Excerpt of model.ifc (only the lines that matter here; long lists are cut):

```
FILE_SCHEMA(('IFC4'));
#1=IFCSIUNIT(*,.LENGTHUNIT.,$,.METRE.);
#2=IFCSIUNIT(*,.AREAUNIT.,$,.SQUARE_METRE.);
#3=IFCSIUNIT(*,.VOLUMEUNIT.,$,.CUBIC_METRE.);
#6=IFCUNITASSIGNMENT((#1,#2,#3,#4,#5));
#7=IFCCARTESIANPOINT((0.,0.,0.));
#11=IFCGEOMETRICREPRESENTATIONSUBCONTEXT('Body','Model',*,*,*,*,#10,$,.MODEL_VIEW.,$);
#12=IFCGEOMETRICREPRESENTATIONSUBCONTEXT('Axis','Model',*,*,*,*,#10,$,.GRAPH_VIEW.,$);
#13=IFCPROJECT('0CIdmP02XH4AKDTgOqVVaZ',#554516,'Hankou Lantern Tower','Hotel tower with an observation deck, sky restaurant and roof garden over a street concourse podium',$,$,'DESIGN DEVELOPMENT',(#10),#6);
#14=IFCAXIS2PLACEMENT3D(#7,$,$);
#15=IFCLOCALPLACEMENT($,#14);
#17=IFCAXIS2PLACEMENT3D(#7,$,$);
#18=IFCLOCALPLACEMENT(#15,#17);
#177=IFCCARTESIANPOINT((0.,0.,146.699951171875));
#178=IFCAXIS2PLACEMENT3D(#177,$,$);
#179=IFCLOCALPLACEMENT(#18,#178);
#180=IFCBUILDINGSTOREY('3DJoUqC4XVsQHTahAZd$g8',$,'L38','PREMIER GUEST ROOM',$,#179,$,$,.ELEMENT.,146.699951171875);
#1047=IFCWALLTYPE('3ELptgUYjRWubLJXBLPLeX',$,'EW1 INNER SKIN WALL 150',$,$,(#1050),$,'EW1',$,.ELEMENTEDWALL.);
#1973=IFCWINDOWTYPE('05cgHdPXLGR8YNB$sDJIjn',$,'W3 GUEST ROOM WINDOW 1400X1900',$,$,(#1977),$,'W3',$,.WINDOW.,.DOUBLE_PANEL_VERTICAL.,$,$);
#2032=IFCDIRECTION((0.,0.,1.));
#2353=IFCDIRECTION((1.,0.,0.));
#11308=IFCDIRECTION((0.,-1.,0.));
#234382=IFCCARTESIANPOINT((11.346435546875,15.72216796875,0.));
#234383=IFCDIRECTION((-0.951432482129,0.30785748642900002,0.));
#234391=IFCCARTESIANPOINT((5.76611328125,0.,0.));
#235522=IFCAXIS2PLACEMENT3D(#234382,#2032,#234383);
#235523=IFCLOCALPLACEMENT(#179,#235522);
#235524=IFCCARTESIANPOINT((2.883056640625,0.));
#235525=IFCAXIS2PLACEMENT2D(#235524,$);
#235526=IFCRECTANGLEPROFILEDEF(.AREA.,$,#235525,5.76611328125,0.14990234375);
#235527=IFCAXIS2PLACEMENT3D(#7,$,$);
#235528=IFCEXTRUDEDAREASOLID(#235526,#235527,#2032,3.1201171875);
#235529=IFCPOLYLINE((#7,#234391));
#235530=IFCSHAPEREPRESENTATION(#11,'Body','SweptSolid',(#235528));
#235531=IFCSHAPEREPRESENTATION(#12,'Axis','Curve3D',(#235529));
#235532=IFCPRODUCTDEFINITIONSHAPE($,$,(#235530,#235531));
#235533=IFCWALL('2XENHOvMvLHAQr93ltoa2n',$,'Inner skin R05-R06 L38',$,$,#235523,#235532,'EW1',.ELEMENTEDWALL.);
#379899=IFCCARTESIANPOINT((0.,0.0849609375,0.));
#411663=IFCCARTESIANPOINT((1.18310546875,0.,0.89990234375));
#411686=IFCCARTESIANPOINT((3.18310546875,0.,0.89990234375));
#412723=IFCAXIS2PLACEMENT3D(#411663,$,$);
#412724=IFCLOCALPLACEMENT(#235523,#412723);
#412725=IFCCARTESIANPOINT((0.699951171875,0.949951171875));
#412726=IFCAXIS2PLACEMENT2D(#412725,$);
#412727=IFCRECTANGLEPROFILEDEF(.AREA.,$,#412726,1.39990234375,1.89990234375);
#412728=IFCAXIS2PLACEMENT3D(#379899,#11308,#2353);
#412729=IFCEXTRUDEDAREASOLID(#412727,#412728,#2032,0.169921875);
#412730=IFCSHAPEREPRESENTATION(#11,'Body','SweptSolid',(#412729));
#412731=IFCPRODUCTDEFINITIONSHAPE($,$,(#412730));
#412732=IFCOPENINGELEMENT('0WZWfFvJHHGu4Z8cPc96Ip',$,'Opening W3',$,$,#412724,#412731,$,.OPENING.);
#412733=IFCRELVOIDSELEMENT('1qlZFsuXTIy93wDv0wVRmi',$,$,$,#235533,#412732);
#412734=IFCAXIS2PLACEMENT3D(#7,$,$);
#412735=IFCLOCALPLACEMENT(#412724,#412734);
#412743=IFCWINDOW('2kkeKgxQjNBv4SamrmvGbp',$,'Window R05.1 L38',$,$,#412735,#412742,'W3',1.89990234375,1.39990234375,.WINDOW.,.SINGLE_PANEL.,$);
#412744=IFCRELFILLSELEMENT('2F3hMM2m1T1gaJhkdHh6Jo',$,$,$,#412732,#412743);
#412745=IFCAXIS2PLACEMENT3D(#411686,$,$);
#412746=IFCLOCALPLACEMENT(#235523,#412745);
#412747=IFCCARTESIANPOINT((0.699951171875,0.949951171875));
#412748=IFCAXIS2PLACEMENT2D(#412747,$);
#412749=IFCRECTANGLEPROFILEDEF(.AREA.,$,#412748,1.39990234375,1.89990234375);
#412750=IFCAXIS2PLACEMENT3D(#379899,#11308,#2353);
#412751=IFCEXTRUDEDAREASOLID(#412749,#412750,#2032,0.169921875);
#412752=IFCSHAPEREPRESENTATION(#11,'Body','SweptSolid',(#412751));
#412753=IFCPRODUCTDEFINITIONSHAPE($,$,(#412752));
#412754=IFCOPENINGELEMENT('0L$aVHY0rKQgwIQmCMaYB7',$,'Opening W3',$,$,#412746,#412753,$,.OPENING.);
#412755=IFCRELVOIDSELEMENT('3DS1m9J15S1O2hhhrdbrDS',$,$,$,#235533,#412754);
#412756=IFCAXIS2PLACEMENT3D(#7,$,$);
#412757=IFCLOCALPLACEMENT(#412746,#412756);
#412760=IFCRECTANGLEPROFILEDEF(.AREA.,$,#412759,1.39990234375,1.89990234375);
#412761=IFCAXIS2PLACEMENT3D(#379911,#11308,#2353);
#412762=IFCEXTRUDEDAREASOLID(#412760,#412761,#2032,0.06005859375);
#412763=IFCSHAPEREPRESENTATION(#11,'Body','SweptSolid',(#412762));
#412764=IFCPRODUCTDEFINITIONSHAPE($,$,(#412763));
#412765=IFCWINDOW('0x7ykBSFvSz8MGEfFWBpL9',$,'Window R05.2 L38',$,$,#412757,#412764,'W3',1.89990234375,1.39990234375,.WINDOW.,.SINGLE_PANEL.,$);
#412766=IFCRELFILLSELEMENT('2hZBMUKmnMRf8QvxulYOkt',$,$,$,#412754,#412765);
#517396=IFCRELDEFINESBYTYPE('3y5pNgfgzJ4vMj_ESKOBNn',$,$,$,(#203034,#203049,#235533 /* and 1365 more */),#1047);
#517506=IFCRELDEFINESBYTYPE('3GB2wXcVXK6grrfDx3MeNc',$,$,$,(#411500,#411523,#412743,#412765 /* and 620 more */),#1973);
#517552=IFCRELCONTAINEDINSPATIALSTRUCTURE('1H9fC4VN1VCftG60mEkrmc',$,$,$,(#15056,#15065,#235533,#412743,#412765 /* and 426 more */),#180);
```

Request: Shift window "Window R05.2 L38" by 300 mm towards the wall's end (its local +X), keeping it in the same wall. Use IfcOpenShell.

```python
import ifcopenshell
import ifcopenshell.api.geometry
import ifcopenshell.util.placement
import ifcopenshell.util.unit

model = ifcopenshell.open("model.ifc")
unit_scale = ifcopenshell.util.unit.calculate_unit_scale(model)

window = model.by_guid("0x7ykBSFvSz8MGEfFWBpL9")
opening = window.FillsVoids[0].RelatingOpeningElement
wall = opening.VoidsElements[0].RelatingBuildingElement

wall_matrix = ifcopenshell.util.placement.get_local_placement(wall.ObjectPlacement)
shift = wall_matrix[:3, 0] * 0.3 / unit_scale
before = ifcopenshell.util.placement.get_local_placement(window.ObjectPlacement)[:3, 3].copy()

# The window is placed relative to its opening, so it follows when the opening moves.
matrix = ifcopenshell.util.placement.get_local_placement(opening.ObjectPlacement)
matrix[:3, 3] += shift
ifcopenshell.api.geometry.edit_object_placement(
    model, product=opening, matrix=matrix, is_si=False, should_transform_children=True
)

after = ifcopenshell.util.placement.get_local_placement(window.ObjectPlacement)[:3, 3]
print("window moved by", (after - before).round(3) + 0.0)

model.write("model_edited.ifc")
```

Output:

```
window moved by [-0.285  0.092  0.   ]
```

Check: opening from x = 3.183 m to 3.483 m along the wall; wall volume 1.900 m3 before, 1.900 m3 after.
